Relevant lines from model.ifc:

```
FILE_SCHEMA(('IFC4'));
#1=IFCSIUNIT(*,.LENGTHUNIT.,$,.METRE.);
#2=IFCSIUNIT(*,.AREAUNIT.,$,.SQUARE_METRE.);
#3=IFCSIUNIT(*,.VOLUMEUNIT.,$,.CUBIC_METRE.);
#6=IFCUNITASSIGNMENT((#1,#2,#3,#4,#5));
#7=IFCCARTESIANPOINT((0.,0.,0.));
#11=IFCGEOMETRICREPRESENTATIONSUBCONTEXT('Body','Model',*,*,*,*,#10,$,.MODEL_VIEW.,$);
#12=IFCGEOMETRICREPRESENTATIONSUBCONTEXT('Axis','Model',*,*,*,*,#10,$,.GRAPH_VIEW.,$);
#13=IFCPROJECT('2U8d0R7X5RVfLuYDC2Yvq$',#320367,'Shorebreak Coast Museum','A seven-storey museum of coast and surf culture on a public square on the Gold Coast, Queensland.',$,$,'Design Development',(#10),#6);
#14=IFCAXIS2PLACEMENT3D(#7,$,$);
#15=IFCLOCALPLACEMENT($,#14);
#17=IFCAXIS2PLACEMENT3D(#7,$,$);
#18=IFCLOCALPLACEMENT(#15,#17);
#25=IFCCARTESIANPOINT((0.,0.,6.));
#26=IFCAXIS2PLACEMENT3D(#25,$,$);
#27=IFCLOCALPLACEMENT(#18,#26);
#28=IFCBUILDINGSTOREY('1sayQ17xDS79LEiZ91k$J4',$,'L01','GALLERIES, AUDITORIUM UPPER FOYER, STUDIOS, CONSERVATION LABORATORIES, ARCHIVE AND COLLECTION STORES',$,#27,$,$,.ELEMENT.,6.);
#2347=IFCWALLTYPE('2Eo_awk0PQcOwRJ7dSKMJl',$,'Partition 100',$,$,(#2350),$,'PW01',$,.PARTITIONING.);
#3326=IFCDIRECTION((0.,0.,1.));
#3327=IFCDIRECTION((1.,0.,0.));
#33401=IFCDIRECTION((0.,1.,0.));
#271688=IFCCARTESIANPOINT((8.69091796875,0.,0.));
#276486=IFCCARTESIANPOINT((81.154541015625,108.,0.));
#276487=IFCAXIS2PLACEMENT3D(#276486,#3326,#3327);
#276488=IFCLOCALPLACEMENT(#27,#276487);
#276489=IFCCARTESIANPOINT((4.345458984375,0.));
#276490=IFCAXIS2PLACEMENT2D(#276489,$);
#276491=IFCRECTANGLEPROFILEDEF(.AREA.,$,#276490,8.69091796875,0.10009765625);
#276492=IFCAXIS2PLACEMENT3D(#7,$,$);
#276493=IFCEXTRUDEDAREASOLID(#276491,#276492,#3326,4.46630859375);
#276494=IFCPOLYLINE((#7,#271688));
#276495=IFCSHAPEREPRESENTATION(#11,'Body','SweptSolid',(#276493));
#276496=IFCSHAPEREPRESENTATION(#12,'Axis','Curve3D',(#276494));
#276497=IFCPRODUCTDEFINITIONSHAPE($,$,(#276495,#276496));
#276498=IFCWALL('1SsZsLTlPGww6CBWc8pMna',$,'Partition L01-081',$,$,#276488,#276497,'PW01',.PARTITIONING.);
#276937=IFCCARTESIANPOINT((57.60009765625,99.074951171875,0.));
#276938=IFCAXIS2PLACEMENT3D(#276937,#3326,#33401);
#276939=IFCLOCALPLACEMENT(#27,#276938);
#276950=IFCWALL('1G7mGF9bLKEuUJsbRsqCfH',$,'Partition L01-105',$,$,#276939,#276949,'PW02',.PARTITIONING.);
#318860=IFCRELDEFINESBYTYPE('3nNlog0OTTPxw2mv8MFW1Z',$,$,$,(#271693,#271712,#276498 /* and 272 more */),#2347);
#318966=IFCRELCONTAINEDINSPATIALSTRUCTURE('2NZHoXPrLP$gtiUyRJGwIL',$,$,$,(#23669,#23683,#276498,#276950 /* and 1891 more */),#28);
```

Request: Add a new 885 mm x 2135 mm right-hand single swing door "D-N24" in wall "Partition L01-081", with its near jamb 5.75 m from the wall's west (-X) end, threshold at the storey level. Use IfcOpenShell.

```python
import numpy as np
import ifcopenshell
import ifcopenshell.api.feature
import ifcopenshell.api.geometry
import ifcopenshell.api.root
import ifcopenshell.api.spatial
import ifcopenshell.geom
import ifcopenshell.util.element
import ifcopenshell.util.placement
import ifcopenshell.util.representation
import ifcopenshell.util.shape
import ifcopenshell.util.unit

model = ifcopenshell.open("model.ifc")
unit_scale = ifcopenshell.util.unit.calculate_unit_scale(model)
settings = ifcopenshell.geom.settings()


def volume(element):
    """Net volume in cubic metres, openings subtracted."""
    shape = ifcopenshell.geom.create_shape(settings, element)
    return ifcopenshell.util.shape.get_volume(shape.geometry)


wall = model.by_guid("1SsZsLTlPGww6CBWc8pMna")
storey = ifcopenshell.util.element.get_container(wall, ifc_class="IfcBuildingStorey")
context = ifcopenshell.util.representation.get_context(model, "Model", "Body", "MODEL_VIEW")
before = volume(wall)

width, height, from_end, sill = 0.885, 2.135, 5.75, 0.0  # metres

# The wall runs along its own X axis, and the end named is its -X end.
wall_shape = ifcopenshell.geom.create_shape(settings, wall)
x, y, z = ifcopenshell.util.shape.get_vertices(wall_shape.geometry).T
start = x.min() + from_end
face, thickness = float(y.min()), float(y.max() - y.min())
wall_matrix = ifcopenshell.util.placement.get_local_placement(wall.ObjectPlacement)
level = ifcopenshell.util.placement.get_local_placement(storey.ObjectPlacement)[2, 3]


def in_wall(x, y):
    """Placement at x, y metres in the wall's axes, at sill height."""
    matrix = wall_matrix.copy()
    matrix[:, 3] = wall_matrix @ np.array([x / unit_scale, y / unit_scale, 0.0, 1.0])
    matrix[2, 3] = level + sill / unit_scale
    return matrix


# Opening: a box that overshoots both wall faces by 50 mm.
opening = ifcopenshell.api.root.create_entity(model, ifc_class="IfcOpeningElement", predefined_type="OPENING")
box = ifcopenshell.api.geometry.add_wall_representation(
    model, context=context, length=width, height=height, thickness=thickness + 0.1
)
ifcopenshell.api.geometry.assign_representation(model, product=opening, representation=box)
ifcopenshell.api.geometry.edit_object_placement(model, product=opening, matrix=in_wall(start, face - 0.05), is_si=False)
ifcopenshell.api.feature.add_feature(model, feature=opening, element=wall)

door = ifcopenshell.api.root.create_entity(model, ifc_class="IfcDoor", name="D-N24", predefined_type="DOOR")
door.OverallWidth, door.OverallHeight = width / unit_scale, height / unit_scale
door.OperationType = "SINGLE_SWING_RIGHT"
body = ifcopenshell.api.geometry.add_door_representation(
    model,
    context=context,
    overall_width=door.OverallWidth,
    overall_height=door.OverallHeight,
    operation_type="SINGLE_SWING_RIGHT",
    lining_properties={"LiningDepth": thickness / unit_scale, "ThresholdDepth": thickness / unit_scale},
)
ifcopenshell.api.geometry.assign_representation(model, product=door, representation=body)
ifcopenshell.api.spatial.assign_container(model, products=[door], relating_structure=storey)
ifcopenshell.api.feature.add_filling(model, opening=opening, element=door)

# The lining spans the wall, so the door starts at the wall face.
ifcopenshell.api.geometry.edit_object_placement(model, product=door, matrix=in_wall(start, face), is_si=False)

after = volume(wall)

print(f"wall volume {before:.3f} -> {after:.3f} m3")

model.write("model_rev.ifc")
```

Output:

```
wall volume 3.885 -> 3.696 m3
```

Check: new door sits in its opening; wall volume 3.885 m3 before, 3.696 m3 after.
